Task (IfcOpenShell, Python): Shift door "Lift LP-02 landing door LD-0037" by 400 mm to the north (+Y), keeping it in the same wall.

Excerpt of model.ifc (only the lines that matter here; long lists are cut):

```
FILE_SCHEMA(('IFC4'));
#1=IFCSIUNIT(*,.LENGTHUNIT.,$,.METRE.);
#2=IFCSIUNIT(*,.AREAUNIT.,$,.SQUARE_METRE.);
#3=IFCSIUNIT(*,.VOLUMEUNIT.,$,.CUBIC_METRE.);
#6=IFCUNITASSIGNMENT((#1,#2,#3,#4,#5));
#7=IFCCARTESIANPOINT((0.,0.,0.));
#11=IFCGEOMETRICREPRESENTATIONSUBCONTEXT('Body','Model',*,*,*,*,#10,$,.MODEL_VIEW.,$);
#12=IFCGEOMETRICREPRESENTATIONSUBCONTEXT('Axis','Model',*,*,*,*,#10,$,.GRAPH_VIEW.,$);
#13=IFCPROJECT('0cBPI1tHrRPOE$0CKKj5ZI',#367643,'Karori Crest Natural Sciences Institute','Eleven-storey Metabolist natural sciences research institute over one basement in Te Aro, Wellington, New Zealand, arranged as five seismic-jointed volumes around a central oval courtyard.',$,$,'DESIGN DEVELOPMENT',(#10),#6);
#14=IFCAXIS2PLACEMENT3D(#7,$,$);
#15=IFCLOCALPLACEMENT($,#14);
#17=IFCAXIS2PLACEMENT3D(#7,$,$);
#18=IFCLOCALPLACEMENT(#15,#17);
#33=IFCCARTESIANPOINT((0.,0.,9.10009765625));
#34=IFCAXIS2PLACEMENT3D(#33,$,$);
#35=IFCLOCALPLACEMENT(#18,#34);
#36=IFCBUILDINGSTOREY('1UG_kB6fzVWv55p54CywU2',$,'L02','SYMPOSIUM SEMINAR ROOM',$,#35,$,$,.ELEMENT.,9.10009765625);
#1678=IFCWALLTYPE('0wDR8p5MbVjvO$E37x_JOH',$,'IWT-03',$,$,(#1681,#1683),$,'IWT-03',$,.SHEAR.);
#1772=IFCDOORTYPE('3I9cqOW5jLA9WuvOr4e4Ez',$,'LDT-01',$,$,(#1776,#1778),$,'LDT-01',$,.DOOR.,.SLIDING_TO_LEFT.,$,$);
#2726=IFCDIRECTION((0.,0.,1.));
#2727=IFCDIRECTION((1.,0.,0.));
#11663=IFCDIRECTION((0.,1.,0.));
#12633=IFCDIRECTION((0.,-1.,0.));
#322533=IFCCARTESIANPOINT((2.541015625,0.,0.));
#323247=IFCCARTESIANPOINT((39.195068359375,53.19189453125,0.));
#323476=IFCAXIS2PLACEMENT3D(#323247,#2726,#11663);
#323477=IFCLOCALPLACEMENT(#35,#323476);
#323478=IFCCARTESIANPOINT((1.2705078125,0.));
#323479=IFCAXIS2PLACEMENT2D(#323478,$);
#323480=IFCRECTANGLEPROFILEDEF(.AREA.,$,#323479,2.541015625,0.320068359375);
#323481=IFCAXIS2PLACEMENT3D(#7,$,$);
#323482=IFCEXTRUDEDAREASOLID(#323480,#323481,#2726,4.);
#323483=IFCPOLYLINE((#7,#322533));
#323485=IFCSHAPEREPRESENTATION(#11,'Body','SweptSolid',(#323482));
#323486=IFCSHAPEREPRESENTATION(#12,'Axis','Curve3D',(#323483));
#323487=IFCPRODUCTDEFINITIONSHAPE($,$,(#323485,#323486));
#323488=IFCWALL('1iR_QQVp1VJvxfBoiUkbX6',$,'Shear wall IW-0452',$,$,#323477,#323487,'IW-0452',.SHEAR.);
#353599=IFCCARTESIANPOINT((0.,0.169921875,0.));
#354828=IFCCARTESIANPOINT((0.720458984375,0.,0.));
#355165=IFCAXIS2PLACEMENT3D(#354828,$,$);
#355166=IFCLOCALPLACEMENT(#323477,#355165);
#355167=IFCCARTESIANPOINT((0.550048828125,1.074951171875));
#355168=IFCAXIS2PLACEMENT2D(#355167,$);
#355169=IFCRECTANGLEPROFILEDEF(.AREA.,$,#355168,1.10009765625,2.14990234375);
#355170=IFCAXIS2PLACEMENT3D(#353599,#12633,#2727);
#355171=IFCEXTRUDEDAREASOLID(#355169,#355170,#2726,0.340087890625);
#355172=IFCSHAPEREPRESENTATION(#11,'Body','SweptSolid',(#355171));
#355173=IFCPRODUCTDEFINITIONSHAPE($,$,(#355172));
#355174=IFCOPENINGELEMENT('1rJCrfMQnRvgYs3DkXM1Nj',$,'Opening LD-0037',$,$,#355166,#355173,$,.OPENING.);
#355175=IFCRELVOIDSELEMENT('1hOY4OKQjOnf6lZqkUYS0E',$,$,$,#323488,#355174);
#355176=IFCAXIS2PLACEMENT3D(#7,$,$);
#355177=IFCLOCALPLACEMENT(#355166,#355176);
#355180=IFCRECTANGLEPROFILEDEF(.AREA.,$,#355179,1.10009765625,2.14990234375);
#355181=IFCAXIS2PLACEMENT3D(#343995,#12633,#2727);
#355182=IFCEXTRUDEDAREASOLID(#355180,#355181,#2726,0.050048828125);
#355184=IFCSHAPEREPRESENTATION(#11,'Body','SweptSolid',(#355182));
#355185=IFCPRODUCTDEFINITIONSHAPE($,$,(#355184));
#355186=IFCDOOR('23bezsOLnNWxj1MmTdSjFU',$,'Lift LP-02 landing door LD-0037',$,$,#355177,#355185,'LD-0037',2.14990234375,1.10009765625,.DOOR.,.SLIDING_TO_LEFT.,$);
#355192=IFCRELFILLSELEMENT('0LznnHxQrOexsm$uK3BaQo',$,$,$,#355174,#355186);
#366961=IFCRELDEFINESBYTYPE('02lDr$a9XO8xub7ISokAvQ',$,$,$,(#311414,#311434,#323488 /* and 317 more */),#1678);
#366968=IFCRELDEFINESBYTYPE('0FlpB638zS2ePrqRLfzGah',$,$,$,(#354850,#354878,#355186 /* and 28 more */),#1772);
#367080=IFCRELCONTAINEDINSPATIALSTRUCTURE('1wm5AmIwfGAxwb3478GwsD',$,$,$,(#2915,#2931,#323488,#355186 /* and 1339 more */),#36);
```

```python
import ifcopenshell
import ifcopenshell.api.geometry
import ifcopenshell.util.placement

model = ifcopenshell.open("model.ifc")

door = model.by_id(355186)
opening = door.FillsVoids[0].RelatingOpeningElement
wall = opening.VoidsElements[0].RelatingBuildingElement

wall_matrix = ifcopenshell.util.placement.get_local_placement(wall.ObjectPlacement)
shift = wall_matrix[:3, 0] * 0.4
before = ifcopenshell.util.placement.get_local_placement(door.ObjectPlacement)[:3, 3].copy()

# The door is placed relative to its opening, so it follows when the opening moves.
matrix = ifcopenshell.util.placement.get_local_placement(opening.ObjectPlacement)
matrix[:3, 3] += shift
ifcopenshell.api.geometry.edit_object_placement(
    model, product=opening, matrix=matrix, is_si=False, should_transform_children=True
)

after = ifcopenshell.util.placement.get_local_placement(door.ObjectPlacement)[:3, 3]
print("door moved by", (after - before).round(3) + 0.0)

model.write("model-out.ifc")
```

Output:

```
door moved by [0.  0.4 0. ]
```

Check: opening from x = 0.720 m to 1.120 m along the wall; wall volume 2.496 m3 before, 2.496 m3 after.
